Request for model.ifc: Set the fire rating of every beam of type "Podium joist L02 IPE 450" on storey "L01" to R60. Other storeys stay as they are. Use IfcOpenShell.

First a look at what the model holds.

```python
import ifcopenshell
import ifcopenshell.util.element

model = ifcopenshell.open("model.ifc")
print(model.schema)
storey = next(s for s in model.by_type("IfcBuildingStorey") if s.Name == "L01")
beams = [e for e in ifcopenshell.util.element.get_decomposition(storey) if e.is_a("IfcBeam")]
seen = {}
for e in beams:
    element_type = ifcopenshell.util.element.get_type(e)
    key = (element_type.Name if element_type != e and element_type else None, ifcopenshell.util.element.get_pset(e, "Pset_BeamCommon", "FireRating"))
    seen[key] = seen.get(key, 0) + 1
for (name, value), count in sorted(seen.items(), key=str):
    print(count, "x", name, "|", value)
```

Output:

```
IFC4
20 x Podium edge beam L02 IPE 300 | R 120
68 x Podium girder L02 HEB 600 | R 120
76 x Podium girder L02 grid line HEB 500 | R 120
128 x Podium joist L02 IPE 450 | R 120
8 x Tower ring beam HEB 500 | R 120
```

```python
import ifcopenshell
import ifcopenshell.api.pset
import ifcopenshell.util.element

model = ifcopenshell.open("model.ifc")

storey = next(s for s in model.by_type("IfcBuildingStorey") if s.Name == "L01")
beams = [e for e in ifcopenshell.util.element.get_decomposition(storey) if e.is_a("IfcBeam")]

count = 0
for e in beams:
    element_type = ifcopenshell.util.element.get_type(e)
    if element_type in (None, e) or element_type.Name != "Podium joist L02 IPE 450":
        continue
    found = ifcopenshell.util.element.get_pset(e, "Pset_BeamCommon", should_inherit=False)
    if found:
        pset = model.by_id(found["id"])
        if len(ifcopenshell.util.element.get_elements_by_pset(pset)) > 1:
            pset = ifcopenshell.api.pset.unshare_pset(model, products=[e], pset=pset)[0]
    else:
        pset = ifcopenshell.api.pset.add_pset(model, product=e, name="Pset_BeamCommon")
    ifcopenshell.api.pset.edit_pset(model, pset=pset, properties={"FireRating": "R60"})
    count += 1

print(count, "beams updated")

model.write("model_edited.ifc")
```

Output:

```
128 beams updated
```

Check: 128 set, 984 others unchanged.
